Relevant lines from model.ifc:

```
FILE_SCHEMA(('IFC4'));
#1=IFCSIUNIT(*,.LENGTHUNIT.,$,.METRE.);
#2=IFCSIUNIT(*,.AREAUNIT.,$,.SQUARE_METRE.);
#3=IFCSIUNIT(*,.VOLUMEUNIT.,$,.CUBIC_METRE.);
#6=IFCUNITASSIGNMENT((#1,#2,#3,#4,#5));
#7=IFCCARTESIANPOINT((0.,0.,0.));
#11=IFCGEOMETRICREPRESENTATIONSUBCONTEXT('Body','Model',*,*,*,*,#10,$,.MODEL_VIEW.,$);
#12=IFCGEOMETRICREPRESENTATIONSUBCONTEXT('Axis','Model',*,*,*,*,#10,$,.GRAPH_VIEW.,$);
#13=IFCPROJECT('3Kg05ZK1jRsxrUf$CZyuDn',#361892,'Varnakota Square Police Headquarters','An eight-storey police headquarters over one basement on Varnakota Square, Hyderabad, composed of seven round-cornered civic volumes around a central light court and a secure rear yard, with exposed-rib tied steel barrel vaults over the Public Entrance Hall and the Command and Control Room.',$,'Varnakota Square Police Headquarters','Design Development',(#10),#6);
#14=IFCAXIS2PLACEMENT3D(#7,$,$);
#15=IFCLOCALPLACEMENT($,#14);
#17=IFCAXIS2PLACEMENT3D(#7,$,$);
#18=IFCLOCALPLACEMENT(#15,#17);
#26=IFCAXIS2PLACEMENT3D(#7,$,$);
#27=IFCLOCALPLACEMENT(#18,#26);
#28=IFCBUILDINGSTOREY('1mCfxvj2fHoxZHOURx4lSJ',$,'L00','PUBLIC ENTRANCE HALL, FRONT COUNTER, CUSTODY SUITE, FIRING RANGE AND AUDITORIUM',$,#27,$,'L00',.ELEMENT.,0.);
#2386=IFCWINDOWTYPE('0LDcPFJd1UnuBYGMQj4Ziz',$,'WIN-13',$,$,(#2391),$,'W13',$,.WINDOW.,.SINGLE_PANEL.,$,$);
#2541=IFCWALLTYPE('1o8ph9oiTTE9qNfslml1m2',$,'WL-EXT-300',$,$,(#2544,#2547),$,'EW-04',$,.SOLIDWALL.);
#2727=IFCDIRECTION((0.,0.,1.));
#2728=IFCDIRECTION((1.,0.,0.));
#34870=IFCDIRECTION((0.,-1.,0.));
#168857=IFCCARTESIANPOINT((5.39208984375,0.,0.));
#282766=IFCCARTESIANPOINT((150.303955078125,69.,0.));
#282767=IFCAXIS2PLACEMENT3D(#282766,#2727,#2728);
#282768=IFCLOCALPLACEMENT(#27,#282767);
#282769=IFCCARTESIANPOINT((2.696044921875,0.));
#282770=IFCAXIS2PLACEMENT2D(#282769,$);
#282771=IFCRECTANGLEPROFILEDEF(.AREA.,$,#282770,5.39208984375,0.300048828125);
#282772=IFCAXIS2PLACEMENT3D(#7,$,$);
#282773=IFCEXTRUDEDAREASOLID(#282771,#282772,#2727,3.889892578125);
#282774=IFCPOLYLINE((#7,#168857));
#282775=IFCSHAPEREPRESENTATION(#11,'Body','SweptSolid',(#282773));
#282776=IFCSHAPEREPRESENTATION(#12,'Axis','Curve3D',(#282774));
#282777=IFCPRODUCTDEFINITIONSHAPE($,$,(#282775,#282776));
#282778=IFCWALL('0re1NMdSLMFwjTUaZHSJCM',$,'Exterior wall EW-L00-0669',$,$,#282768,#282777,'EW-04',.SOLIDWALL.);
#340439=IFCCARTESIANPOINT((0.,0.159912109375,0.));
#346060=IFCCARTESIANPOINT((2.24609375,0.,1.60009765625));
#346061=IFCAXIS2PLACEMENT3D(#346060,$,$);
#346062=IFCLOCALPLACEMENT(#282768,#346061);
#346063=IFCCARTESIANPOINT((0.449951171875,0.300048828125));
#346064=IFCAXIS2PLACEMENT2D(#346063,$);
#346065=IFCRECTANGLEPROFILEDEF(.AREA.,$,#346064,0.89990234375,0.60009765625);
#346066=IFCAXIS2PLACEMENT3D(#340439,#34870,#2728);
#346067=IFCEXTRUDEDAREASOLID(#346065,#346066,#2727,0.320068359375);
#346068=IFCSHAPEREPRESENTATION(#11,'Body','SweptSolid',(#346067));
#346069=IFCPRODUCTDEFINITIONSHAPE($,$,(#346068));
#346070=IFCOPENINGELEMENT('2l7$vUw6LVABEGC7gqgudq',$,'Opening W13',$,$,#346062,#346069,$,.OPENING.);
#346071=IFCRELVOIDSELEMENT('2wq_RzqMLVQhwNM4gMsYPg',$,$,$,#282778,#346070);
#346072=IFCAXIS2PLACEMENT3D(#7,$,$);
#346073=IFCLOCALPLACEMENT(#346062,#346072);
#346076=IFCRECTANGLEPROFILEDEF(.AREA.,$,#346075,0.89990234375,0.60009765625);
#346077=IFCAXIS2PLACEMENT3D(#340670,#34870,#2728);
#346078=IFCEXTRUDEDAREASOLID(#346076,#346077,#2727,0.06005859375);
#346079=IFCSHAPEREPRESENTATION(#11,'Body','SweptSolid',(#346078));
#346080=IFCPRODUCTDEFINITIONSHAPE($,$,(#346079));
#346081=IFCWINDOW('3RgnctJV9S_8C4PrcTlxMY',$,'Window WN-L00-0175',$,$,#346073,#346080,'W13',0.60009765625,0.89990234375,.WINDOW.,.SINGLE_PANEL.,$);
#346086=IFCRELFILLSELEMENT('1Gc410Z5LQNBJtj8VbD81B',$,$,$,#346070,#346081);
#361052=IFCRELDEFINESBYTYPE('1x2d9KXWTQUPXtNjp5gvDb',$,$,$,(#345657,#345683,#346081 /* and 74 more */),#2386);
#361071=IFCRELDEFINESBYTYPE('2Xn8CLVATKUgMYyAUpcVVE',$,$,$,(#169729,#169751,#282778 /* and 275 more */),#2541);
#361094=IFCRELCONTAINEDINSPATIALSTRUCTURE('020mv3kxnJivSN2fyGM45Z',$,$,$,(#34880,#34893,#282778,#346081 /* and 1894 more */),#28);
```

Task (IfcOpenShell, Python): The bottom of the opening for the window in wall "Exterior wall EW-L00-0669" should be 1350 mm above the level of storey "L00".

```python
import numpy as np
import ifcopenshell
import ifcopenshell.api.geometry
import ifcopenshell.geom
import ifcopenshell.util.element
import ifcopenshell.util.placement
import ifcopenshell.util.shape
import ifcopenshell.util.unit

model = ifcopenshell.open("model.ifc")
unit_scale = ifcopenshell.util.unit.calculate_unit_scale(model)

window = model.by_guid("3RgnctJV9S_8C4PrcTlxMY")
opening = window.FillsVoids[0].RelatingOpeningElement
storey = ifcopenshell.util.element.get_container(window, ifc_class="IfcBuildingStorey")
level = ifcopenshell.util.placement.get_local_placement(storey.ObjectPlacement)[2, 3]

# The opening's origin need not be at the sill, so measure its lowest point.
shape = ifcopenshell.geom.create_shape(ifcopenshell.geom.settings(), opening)
bottom = ifcopenshell.util.shape.get_shape_bottom_elevation(shape, shape.geometry) / unit_scale
dz = level + 1.35 / unit_scale - bottom

shift = np.array([0.0, 0.0, dz])
# The window is placed relative to its opening, so it follows when the opening moves.
matrix = ifcopenshell.util.placement.get_local_placement(opening.ObjectPlacement)
matrix[:3, 3] += shift
ifcopenshell.api.geometry.edit_object_placement(
    model, product=opening, matrix=matrix, is_si=False, should_transform_children=True
)

print(f"moved by {dz * unit_scale:+.3f} m")

model.write("model_edited.ifc")
```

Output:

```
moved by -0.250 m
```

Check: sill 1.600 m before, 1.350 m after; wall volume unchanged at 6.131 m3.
